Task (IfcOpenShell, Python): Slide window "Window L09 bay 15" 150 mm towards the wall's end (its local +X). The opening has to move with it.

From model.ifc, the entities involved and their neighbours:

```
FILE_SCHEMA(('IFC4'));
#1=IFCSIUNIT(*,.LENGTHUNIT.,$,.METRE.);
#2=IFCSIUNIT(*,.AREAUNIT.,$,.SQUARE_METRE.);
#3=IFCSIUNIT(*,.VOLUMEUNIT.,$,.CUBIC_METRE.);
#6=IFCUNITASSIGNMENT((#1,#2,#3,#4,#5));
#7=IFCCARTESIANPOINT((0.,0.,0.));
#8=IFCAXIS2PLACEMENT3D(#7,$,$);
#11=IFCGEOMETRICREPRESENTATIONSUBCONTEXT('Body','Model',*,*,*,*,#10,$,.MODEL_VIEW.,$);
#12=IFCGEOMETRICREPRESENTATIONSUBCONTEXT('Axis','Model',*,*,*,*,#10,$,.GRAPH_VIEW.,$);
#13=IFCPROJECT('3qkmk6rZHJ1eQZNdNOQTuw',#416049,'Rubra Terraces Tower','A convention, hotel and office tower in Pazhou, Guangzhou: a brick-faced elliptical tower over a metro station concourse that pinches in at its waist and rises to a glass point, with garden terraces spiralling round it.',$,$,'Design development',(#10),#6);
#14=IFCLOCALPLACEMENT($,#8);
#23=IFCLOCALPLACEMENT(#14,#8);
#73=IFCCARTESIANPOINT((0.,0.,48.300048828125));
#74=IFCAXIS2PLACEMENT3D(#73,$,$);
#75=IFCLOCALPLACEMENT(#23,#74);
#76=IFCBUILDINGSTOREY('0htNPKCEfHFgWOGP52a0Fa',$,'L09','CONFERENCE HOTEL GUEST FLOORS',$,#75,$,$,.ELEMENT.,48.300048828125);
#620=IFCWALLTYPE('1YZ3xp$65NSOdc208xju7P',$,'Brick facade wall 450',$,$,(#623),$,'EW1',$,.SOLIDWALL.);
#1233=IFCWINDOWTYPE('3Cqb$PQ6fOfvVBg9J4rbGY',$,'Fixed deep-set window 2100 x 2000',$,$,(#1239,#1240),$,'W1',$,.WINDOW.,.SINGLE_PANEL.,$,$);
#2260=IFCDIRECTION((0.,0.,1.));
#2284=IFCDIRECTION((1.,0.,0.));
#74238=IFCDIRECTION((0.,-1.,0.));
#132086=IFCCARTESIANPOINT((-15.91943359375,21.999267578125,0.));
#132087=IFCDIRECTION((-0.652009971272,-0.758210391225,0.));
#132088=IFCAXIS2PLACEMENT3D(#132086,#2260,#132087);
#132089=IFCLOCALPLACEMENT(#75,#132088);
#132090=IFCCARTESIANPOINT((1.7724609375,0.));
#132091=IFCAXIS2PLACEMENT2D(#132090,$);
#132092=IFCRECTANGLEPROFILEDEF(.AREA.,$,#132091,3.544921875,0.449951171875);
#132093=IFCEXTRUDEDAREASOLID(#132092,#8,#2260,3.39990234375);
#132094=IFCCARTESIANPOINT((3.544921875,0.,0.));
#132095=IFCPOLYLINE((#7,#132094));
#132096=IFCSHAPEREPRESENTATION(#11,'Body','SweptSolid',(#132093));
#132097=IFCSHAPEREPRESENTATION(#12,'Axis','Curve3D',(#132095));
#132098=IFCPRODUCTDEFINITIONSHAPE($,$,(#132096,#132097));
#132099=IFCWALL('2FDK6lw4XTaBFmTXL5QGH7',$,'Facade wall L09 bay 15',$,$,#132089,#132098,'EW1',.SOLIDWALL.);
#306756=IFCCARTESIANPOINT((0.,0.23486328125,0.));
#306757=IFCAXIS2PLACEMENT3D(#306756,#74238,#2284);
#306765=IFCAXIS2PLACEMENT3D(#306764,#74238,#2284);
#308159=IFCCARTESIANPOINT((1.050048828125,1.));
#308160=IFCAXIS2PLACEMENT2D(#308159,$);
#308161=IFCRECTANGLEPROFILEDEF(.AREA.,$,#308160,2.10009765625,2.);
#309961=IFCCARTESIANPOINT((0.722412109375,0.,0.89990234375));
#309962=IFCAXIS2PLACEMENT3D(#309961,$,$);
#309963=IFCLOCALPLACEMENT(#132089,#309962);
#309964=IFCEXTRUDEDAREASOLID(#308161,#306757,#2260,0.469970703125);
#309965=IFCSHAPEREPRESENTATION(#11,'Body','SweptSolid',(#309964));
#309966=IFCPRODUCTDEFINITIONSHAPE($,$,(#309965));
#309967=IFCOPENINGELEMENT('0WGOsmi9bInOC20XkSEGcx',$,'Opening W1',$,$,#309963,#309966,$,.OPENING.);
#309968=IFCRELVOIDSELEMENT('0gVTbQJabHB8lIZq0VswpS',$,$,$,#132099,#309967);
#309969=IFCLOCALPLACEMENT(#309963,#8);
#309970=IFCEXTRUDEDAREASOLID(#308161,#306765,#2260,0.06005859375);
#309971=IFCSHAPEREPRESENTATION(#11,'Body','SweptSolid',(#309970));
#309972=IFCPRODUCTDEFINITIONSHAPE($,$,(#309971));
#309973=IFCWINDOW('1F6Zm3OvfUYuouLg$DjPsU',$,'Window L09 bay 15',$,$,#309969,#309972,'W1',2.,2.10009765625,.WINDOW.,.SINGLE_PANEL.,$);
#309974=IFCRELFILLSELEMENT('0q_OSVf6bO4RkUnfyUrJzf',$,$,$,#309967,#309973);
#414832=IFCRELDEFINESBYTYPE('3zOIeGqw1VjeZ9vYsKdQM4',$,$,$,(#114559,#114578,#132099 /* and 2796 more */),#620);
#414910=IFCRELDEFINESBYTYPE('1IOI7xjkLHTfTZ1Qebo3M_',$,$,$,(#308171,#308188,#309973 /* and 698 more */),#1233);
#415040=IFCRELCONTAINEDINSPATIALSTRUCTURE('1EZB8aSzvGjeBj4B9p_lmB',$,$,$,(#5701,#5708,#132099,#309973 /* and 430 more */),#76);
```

```python
import ifcopenshell
import ifcopenshell.api.geometry
import ifcopenshell.util.placement
import ifcopenshell.util.unit

model = ifcopenshell.open("model.ifc")
unit_scale = ifcopenshell.util.unit.calculate_unit_scale(model)

window = model.by_id(309973)
opening = window.FillsVoids[0].RelatingOpeningElement
wall = opening.VoidsElements[0].RelatingBuildingElement

wall_matrix = ifcopenshell.util.placement.get_local_placement(wall.ObjectPlacement)
shift = wall_matrix[:3, 0] * 0.15 / unit_scale
before = ifcopenshell.util.placement.get_local_placement(window.ObjectPlacement)[:3, 3].copy()

# The window is placed relative to its opening, so it follows when the opening moves.
matrix = ifcopenshell.util.placement.get_local_placement(opening.ObjectPlacement)
matrix[:3, 3] += shift
ifcopenshell.api.geometry.edit_object_placement(
    model, product=opening, matrix=matrix, is_si=False, should_transform_children=True
)

after = ifcopenshell.util.placement.get_local_placement(window.ObjectPlacement)[:3, 3]
print("window moved by", (after - before).round(3) + 0.0)

model.write("model_edited.ifc")
```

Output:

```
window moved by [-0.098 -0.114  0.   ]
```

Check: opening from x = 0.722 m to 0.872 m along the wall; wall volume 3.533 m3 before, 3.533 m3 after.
